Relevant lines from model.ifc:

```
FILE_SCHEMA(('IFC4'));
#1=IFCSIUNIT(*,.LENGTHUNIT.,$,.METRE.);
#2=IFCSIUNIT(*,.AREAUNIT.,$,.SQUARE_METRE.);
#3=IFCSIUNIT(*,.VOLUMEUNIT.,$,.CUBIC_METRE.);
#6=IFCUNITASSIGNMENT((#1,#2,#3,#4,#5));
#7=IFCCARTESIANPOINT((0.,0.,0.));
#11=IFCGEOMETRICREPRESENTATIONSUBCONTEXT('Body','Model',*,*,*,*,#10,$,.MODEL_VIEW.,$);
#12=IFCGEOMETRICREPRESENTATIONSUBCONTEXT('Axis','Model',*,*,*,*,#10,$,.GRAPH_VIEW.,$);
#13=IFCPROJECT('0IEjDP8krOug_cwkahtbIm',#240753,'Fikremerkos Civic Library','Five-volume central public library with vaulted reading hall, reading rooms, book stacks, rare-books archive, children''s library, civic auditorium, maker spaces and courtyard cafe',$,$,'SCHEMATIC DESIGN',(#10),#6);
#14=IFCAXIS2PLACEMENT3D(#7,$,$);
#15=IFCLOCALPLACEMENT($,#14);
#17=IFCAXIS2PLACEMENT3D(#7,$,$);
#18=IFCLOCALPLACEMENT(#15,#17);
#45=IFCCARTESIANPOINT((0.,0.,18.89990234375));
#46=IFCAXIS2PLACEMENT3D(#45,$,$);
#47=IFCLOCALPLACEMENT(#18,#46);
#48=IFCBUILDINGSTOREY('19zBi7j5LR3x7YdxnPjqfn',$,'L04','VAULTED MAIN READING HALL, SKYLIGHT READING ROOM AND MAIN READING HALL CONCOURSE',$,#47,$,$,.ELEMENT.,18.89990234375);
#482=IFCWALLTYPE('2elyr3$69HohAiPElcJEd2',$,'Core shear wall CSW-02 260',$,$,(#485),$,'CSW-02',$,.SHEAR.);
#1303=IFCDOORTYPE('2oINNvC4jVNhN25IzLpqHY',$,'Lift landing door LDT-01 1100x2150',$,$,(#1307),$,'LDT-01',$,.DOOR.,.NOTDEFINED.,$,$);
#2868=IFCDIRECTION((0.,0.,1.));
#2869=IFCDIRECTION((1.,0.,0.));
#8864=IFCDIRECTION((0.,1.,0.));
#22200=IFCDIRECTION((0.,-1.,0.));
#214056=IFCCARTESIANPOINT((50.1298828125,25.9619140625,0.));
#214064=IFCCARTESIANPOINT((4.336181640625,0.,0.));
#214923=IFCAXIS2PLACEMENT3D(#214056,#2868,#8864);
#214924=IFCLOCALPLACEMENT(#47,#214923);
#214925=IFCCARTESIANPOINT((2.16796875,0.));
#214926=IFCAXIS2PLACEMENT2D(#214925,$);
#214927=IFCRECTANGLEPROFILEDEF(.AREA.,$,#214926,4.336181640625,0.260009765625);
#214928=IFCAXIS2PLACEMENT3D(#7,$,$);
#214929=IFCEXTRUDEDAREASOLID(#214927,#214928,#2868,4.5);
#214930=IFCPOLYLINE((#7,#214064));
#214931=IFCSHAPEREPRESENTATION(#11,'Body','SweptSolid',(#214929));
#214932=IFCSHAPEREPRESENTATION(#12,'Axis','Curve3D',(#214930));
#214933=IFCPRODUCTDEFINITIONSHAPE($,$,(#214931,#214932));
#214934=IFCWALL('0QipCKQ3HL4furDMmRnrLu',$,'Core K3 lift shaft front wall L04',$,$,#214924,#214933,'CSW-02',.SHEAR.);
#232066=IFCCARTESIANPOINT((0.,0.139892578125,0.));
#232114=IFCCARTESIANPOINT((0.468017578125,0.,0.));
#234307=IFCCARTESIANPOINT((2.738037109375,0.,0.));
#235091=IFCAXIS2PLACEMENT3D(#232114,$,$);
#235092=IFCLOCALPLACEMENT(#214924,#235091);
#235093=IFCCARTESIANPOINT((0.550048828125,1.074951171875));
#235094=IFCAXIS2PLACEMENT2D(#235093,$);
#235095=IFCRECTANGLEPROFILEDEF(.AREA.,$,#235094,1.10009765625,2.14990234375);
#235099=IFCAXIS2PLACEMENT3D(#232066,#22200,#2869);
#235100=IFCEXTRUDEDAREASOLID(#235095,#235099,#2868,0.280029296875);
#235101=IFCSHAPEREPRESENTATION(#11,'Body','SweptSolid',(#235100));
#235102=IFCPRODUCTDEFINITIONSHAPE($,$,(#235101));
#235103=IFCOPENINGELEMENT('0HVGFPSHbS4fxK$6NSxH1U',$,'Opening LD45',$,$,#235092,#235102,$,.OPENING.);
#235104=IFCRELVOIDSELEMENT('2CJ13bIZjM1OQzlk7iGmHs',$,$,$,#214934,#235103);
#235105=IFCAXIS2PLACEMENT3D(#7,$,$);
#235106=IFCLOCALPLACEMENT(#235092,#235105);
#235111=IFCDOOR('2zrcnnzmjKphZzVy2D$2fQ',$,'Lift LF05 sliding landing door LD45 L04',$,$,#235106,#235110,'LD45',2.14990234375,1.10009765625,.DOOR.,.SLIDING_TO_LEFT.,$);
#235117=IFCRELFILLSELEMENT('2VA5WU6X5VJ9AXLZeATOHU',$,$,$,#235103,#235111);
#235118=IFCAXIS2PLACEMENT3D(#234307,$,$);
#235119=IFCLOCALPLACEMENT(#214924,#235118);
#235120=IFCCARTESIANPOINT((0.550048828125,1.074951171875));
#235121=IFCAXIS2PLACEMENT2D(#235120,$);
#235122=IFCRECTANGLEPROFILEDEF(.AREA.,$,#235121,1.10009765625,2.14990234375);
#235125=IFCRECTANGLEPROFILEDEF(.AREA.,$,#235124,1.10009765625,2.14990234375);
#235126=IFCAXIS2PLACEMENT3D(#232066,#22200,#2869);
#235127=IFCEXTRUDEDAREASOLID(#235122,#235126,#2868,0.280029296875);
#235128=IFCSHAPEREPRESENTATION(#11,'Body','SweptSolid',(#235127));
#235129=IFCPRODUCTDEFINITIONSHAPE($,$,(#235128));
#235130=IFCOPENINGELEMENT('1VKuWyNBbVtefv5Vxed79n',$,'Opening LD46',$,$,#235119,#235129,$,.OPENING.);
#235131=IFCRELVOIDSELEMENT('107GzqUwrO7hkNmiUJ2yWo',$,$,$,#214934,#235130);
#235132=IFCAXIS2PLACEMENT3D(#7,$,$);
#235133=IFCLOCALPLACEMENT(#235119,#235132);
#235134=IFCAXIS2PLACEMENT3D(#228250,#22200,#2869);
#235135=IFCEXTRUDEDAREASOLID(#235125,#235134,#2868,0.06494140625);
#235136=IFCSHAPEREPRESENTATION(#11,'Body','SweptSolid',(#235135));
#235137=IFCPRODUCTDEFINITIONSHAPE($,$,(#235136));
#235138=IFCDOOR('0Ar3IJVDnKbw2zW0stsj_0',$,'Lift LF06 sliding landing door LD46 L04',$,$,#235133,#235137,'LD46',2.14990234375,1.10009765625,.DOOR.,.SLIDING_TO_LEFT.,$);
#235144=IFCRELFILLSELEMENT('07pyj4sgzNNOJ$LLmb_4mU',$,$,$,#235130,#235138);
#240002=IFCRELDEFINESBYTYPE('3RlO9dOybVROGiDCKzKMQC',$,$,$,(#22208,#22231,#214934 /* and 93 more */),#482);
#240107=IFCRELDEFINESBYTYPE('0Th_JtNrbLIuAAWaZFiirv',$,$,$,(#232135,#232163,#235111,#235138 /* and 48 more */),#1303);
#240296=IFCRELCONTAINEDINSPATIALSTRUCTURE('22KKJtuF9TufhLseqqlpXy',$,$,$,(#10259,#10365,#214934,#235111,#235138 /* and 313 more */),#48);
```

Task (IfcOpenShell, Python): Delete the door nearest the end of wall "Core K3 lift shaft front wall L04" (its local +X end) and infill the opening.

```python
import ifcopenshell
import ifcopenshell.api.feature
import ifcopenshell.api.root
import ifcopenshell.geom
import ifcopenshell.util.shape

model = ifcopenshell.open("model.ifc")
settings = ifcopenshell.geom.settings()


def volume(element):
    """Net volume in cubic metres, openings subtracted."""
    shape = ifcopenshell.geom.create_shape(settings, element)
    return ifcopenshell.util.shape.get_volume(shape.geometry)


door = model.by_id(235138)
opening = door.FillsVoids[0].RelatingOpeningElement
wall = opening.VoidsElements[0].RelatingBuildingElement
before = volume(wall)

ifcopenshell.api.root.remove_product(model, product=door)
ifcopenshell.api.feature.remove_feature(model, feature=opening)

after = volume(wall)

print(f"wall volume {before:.3f} -> {after:.3f} m3")

model.write("model_rev.ifc")
```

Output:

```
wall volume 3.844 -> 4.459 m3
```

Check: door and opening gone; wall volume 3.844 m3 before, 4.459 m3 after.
